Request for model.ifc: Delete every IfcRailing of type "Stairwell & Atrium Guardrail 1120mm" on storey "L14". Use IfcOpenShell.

First a look at what the model holds.

```python
import ifcopenshell
import ifcopenshell.util.element

model = ifcopenshell.open("model.ifc")
print(model.schema)
storey = next(s for s in model.by_type("IfcBuildingStorey") if s.Name == "L14")
railings = [e for e in ifcopenshell.util.element.get_decomposition(storey) if e.is_a("IfcRailing")]
seen = {}
for e in railings:
    element_type = ifcopenshell.util.element.get_type(e)
    name = element_type.Name if element_type not in (None, e) else None
    seen[name] = seen.get(name, 0) + 1
for name, count in sorted(seen.items(), key=str):
    print(count, "x", name)
```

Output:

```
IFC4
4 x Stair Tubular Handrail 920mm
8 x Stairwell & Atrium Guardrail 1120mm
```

```python
import ifcopenshell
import ifcopenshell.api.root
import ifcopenshell.util.element

model = ifcopenshell.open("model.ifc")

storey = next(s for s in model.by_type("IfcBuildingStorey") if s.Name == "L14")
railings = [e for e in ifcopenshell.util.element.get_decomposition(storey) if e.is_a("IfcRailing")]
targets = [e for e in railings if (t := ifcopenshell.util.element.get_type(e)) not in (None, e) and t.Name == "Stairwell & Atrium Guardrail 1120mm"]

for e in targets:
    ifcopenshell.api.root.remove_product(model, product=e)
print(len(targets), "removed")

model.write("model-out.ifc")
```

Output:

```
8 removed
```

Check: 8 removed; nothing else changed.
